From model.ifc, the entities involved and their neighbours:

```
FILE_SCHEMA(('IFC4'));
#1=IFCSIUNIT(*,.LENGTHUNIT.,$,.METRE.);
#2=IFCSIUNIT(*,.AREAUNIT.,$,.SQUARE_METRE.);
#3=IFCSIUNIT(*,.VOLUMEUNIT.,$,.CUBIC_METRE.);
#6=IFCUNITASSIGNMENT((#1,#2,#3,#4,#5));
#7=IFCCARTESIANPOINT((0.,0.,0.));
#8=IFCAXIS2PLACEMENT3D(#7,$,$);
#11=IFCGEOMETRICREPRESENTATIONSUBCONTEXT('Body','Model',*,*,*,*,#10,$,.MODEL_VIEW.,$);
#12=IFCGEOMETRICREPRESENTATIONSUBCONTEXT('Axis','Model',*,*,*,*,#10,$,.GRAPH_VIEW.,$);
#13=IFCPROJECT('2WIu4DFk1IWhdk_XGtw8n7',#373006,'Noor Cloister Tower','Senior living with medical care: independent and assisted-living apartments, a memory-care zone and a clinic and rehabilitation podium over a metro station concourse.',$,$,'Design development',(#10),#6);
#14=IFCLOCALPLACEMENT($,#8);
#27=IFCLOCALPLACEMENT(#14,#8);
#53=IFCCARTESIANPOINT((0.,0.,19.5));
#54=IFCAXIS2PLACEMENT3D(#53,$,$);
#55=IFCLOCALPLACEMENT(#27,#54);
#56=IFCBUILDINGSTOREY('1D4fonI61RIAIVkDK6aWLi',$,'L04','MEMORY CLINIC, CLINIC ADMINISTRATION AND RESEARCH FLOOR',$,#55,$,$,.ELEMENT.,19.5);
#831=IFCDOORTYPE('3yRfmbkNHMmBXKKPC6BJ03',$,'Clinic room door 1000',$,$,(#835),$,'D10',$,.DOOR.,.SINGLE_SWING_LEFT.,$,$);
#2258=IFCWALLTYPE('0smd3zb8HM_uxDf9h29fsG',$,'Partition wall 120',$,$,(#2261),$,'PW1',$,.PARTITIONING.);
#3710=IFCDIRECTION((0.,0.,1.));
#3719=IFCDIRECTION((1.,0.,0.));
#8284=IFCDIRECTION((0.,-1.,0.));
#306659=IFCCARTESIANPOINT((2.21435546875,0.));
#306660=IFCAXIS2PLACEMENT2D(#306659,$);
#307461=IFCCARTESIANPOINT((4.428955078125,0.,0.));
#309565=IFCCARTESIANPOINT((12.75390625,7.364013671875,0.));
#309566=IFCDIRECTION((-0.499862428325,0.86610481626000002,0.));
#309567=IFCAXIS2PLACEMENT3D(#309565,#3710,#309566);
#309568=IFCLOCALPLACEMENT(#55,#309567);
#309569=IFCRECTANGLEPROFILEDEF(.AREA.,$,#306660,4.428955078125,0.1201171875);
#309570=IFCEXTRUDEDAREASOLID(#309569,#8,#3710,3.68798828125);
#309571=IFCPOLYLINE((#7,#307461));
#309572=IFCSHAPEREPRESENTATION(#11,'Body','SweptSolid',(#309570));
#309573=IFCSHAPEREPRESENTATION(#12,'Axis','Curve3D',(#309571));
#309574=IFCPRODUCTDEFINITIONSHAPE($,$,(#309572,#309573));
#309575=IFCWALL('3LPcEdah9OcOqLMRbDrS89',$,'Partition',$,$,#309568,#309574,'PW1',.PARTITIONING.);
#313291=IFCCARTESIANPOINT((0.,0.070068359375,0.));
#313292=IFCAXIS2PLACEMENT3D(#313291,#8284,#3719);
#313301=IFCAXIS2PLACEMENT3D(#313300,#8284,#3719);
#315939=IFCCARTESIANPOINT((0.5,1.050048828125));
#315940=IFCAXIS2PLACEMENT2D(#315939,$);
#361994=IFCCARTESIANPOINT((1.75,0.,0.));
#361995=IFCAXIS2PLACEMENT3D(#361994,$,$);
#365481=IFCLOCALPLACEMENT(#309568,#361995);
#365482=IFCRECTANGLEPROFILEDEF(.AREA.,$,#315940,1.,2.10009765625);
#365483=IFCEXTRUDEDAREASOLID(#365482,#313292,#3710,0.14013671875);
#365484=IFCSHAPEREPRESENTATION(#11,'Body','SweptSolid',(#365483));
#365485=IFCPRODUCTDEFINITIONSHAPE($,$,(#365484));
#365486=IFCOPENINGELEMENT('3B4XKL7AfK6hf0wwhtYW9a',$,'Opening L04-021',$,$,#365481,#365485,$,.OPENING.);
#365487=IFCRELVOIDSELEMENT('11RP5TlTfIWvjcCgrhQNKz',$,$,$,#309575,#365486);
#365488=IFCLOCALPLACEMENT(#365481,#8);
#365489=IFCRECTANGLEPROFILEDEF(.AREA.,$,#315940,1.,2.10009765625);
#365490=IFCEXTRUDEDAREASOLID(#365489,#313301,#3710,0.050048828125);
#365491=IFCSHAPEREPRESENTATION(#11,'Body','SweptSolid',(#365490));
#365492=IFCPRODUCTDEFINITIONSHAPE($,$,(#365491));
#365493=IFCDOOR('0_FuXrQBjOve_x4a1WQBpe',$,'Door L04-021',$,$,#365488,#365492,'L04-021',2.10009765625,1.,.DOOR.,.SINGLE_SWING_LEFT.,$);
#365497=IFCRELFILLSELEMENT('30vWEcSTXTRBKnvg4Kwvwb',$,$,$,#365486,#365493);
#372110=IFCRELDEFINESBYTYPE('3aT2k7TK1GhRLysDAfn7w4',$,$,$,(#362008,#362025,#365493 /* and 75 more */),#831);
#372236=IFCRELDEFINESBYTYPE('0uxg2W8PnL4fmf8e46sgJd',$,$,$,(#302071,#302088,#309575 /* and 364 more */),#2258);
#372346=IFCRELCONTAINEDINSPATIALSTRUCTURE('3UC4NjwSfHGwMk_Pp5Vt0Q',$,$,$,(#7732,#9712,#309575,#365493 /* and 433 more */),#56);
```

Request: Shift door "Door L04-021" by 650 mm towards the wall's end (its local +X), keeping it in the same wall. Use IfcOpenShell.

```python
import ifcopenshell
import ifcopenshell.api.geometry
import ifcopenshell.util.placement
import ifcopenshell.util.unit

model = ifcopenshell.open("model.ifc")
unit_scale = ifcopenshell.util.unit.calculate_unit_scale(model)

door = model.by_guid("0_FuXrQBjOve_x4a1WQBpe")
opening = door.FillsVoids[0].RelatingOpeningElement
wall = opening.VoidsElements[0].RelatingBuildingElement

wall_matrix = ifcopenshell.util.placement.get_local_placement(wall.ObjectPlacement)
shift = wall_matrix[:3, 0] * 0.65 / unit_scale
before = ifcopenshell.util.placement.get_local_placement(door.ObjectPlacement)[:3, 3].copy()

# The door is placed relative to its opening, so it follows when the opening moves.
matrix = ifcopenshell.util.placement.get_local_placement(opening.ObjectPlacement)
matrix[:3, 3] += shift
ifcopenshell.api.geometry.edit_object_placement(
    model, product=opening, matrix=matrix, is_si=False, should_transform_children=True
)

after = ifcopenshell.util.placement.get_local_placement(door.ObjectPlacement)[:3, 3]
print("door moved by", (after - before).round(3) + 0.0)

model.write("model_updated.ifc")
```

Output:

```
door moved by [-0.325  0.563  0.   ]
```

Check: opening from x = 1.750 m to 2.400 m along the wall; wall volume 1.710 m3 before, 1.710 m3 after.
